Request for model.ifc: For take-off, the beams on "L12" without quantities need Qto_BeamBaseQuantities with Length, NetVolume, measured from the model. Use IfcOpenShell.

First a look at what the model holds.

```python
import ifcopenshell
import ifcopenshell.util.element
import ifcopenshell.util.unit

model = ifcopenshell.open("model.ifc")
print(model.schema)
for unit_type in ("LENGTHUNIT", "AREAUNIT", "VOLUMEUNIT"):
    print(unit_type, ifcopenshell.util.unit.calculate_unit_scale(model, unit_type))
storey = next(s for s in model.by_type("IfcBuildingStorey") if s.Name == "L12")
beams = [e for e in ifcopenshell.util.element.get_decomposition(storey) if e.is_a("IfcBeam")]
for e in sorted(beams, key=lambda e: e.id()):
    print(e.id(), e.is_a(), e.Name, list(ifcopenshell.util.element.get_psets(e, qtos_only=True)), sep=" | ")
```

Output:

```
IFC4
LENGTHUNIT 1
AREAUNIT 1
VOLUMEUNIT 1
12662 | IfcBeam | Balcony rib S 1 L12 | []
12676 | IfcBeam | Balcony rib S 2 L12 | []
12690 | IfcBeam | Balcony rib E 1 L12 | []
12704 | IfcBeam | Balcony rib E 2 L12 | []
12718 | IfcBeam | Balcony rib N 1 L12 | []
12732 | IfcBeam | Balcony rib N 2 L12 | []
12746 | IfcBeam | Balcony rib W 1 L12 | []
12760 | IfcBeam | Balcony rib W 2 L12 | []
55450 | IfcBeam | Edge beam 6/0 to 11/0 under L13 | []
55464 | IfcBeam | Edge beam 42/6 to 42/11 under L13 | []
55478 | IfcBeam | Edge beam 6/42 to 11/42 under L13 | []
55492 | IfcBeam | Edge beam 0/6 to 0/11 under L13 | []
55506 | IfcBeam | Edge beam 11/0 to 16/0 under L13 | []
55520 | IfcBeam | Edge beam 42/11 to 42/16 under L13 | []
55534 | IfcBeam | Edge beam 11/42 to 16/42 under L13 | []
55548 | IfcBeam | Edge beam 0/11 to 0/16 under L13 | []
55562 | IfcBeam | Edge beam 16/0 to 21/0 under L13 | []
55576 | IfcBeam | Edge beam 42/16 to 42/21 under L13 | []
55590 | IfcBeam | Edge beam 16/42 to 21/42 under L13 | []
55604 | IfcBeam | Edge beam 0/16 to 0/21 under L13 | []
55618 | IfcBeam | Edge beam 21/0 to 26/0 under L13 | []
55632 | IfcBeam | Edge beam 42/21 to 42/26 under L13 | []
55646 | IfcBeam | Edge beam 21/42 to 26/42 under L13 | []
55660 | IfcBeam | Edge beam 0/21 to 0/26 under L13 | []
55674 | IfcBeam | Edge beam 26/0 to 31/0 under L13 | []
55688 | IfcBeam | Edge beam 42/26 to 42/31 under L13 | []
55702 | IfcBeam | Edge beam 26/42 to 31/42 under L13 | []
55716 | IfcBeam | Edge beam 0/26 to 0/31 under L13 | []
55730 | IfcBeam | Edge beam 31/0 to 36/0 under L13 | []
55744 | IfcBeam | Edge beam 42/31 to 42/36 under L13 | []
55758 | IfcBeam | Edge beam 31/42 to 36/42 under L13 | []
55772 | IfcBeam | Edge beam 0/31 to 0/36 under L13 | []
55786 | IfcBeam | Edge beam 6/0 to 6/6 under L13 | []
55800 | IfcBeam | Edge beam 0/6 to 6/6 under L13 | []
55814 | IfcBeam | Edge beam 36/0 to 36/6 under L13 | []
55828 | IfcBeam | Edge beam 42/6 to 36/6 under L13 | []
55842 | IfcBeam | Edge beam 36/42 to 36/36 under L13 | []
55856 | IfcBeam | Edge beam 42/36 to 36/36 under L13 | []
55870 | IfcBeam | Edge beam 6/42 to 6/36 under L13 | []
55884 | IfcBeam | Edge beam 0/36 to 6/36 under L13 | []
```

```python
import ifcopenshell
import ifcopenshell.api.pset
import ifcopenshell.geom
import ifcopenshell.util.element
import ifcopenshell.util.shape
import ifcopenshell.util.unit

model = ifcopenshell.open("model.ifc")
unit_scale = ifcopenshell.util.unit.calculate_unit_scale(model)
volume_scale = ifcopenshell.util.unit.calculate_unit_scale(model, "VOLUMEUNIT")
settings = ifcopenshell.geom.settings()

storey = next(s for s in model.by_type("IfcBuildingStorey") if s.Name == "L12")
beams = [e for e in ifcopenshell.util.element.get_decomposition(storey) if e.is_a("IfcBeam")]

for e in sorted(beams, key=lambda e: e.id()):
    if ifcopenshell.util.element.get_psets(e, qtos_only=True, should_inherit=False):
        continue
    # Geometry comes back in metres, in the element's own axes.
    shape = ifcopenshell.geom.create_shape(settings, e)
    values = {
        "Length": ifcopenshell.util.shape.get_max_xyz(shape.geometry) / unit_scale,
        "NetVolume": ifcopenshell.util.shape.get_volume(shape.geometry) / volume_scale,
    }
    qto = ifcopenshell.api.pset.add_qto(model, product=e, name="Qto_BeamBaseQuantities")
    ifcopenshell.api.pset.edit_qto(model, qto=qto, properties=values)
    print(e.id(), {k: round(v, 3) for k, v in values.items()})

model.write("model_v2.ifc")
```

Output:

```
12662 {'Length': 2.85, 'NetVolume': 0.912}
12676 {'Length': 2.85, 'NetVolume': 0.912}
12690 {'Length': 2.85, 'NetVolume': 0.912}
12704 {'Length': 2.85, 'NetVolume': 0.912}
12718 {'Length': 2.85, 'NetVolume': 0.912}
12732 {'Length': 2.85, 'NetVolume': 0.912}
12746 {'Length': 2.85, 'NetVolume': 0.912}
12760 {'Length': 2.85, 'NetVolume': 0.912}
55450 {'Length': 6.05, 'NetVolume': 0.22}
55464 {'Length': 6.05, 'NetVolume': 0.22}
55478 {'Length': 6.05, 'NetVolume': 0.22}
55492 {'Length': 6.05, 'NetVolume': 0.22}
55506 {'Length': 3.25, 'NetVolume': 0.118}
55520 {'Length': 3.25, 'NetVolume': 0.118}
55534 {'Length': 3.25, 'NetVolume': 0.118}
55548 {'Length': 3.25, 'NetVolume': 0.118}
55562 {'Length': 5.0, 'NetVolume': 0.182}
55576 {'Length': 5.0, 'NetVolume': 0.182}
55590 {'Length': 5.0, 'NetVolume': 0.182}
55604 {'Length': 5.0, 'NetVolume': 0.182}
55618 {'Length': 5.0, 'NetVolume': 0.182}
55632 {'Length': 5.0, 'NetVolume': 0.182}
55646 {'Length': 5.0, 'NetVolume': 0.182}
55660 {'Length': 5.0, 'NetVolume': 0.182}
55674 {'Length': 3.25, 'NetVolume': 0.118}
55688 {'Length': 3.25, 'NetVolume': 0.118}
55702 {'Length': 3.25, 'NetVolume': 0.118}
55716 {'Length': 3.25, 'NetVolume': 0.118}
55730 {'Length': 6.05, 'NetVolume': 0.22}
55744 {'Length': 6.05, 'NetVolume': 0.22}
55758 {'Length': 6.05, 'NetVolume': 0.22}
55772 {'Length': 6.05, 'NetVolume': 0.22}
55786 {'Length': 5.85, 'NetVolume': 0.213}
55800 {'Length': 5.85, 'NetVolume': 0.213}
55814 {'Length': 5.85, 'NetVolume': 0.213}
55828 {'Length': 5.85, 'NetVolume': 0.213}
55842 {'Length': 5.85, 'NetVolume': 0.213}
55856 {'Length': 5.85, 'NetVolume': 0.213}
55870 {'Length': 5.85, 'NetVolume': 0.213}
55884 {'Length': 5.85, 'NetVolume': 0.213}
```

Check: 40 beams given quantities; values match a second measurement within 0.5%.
